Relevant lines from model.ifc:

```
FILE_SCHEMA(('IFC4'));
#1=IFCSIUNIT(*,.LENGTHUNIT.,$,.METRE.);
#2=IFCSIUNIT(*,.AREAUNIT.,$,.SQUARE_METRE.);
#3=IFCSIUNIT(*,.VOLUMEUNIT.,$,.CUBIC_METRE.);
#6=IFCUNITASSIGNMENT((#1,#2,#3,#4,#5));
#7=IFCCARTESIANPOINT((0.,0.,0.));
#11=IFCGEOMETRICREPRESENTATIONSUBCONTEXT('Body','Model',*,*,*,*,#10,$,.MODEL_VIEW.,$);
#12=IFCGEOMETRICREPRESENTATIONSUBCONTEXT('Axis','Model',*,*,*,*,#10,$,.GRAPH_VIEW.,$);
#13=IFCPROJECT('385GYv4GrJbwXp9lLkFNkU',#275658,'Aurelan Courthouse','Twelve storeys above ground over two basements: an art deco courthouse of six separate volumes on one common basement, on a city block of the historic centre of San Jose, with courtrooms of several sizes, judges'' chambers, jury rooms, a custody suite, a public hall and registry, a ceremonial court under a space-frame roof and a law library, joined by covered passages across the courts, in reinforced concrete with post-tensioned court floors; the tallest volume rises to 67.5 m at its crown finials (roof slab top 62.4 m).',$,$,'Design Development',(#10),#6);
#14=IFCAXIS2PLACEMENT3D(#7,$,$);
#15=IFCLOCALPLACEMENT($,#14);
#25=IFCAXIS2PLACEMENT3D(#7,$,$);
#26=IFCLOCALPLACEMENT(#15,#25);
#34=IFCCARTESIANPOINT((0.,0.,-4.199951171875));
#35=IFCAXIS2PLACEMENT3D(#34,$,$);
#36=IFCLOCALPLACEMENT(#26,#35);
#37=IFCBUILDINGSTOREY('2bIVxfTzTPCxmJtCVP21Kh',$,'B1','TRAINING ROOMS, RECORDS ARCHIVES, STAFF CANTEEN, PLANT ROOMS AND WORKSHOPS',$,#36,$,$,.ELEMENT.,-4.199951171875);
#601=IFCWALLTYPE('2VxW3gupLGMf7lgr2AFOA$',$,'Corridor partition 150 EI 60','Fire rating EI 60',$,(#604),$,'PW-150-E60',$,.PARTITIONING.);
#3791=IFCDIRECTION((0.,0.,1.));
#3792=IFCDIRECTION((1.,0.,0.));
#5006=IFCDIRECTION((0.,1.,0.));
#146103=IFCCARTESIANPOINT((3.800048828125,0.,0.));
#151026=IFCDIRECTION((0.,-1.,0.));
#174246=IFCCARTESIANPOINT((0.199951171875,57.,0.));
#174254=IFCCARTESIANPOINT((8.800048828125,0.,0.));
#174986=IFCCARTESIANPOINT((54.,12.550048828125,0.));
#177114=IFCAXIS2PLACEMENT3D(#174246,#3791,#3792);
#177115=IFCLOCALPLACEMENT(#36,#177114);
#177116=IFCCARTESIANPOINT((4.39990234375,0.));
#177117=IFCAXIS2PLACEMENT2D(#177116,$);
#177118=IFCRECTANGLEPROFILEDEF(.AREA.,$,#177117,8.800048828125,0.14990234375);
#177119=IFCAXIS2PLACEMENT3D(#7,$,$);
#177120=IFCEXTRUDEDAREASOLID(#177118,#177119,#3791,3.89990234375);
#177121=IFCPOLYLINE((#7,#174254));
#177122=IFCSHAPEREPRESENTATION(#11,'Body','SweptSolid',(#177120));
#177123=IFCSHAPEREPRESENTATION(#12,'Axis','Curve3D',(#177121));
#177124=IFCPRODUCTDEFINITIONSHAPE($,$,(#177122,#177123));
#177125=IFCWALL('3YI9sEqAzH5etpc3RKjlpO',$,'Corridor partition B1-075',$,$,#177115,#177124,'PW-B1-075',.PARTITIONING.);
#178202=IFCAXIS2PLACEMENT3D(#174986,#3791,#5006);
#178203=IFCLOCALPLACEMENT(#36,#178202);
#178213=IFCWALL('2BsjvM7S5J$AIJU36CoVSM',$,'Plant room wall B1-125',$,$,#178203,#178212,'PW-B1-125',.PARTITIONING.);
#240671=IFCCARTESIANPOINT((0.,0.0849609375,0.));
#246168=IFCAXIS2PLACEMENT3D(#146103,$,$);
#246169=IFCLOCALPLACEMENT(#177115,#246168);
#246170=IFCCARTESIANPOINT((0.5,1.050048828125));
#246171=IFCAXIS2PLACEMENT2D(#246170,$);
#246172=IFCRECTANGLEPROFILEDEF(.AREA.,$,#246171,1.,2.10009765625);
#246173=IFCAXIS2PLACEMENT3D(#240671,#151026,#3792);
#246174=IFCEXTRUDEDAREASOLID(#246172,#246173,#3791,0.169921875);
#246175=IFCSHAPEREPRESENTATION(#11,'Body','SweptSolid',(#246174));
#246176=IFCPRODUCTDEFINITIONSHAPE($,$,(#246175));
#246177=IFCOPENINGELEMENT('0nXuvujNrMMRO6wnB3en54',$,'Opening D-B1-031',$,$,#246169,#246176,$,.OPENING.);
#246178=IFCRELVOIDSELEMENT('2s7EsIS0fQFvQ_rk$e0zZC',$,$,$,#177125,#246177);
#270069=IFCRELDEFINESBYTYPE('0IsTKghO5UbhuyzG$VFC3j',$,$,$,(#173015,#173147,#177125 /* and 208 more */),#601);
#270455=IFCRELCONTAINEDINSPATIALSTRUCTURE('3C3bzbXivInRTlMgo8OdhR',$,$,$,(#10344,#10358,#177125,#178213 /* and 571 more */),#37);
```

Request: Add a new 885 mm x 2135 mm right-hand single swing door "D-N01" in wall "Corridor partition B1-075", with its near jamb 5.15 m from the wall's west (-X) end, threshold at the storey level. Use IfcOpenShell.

```python
import numpy as np
import ifcopenshell
import ifcopenshell.api.feature
import ifcopenshell.api.geometry
import ifcopenshell.api.root
import ifcopenshell.api.spatial
import ifcopenshell.geom
import ifcopenshell.util.element
import ifcopenshell.util.placement
import ifcopenshell.util.representation
import ifcopenshell.util.shape
import ifcopenshell.util.unit

model = ifcopenshell.open("model.ifc")
unit_scale = ifcopenshell.util.unit.calculate_unit_scale(model)
settings = ifcopenshell.geom.settings()


def volume(element):
    """Net volume in cubic metres, openings subtracted."""
    shape = ifcopenshell.geom.create_shape(settings, element)
    return ifcopenshell.util.shape.get_volume(shape.geometry)


wall = model.by_guid("3YI9sEqAzH5etpc3RKjlpO")
storey = ifcopenshell.util.element.get_container(wall, ifc_class="IfcBuildingStorey")
context = ifcopenshell.util.representation.get_context(model, "Model", "Body", "MODEL_VIEW")
before = volume(wall)

width, height, from_end, sill = 0.885, 2.135, 5.15, 0.0  # metres

# The wall runs along its own X axis, and the end named is its -X end.
wall_shape = ifcopenshell.geom.create_shape(settings, wall)
x, y, z = ifcopenshell.util.shape.get_vertices(wall_shape.geometry).T
start = x.min() + from_end
face, thickness = float(y.min()), float(y.max() - y.min())
wall_matrix = ifcopenshell.util.placement.get_local_placement(wall.ObjectPlacement)
level = ifcopenshell.util.placement.get_local_placement(storey.ObjectPlacement)[2, 3]


def in_wall(x, y):
    """Placement at x, y metres in the wall's axes, at sill height."""
    matrix = wall_matrix.copy()
    matrix[:, 3] = wall_matrix @ np.array([x / unit_scale, y / unit_scale, 0.0, 1.0])
    matrix[2, 3] = level + sill / unit_scale
    return matrix


# Opening: a box that overshoots both wall faces by 50 mm.
opening = ifcopenshell.api.root.create_entity(model, ifc_class="IfcOpeningElement", predefined_type="OPENING")
box = ifcopenshell.api.geometry.add_wall_representation(
    model, context=context, length=width, height=height, thickness=thickness + 0.1
)
ifcopenshell.api.geometry.assign_representation(model, product=opening, representation=box)
ifcopenshell.api.geometry.edit_object_placement(model, product=opening, matrix=in_wall(start, face - 0.05), is_si=False)
ifcopenshell.api.feature.add_feature(model, feature=opening, element=wall)

door = ifcopenshell.api.root.create_entity(model, ifc_class="IfcDoor", name="D-N01", predefined_type="DOOR")
door.OverallWidth, door.OverallHeight = width / unit_scale, height / unit_scale
door.OperationType = "SINGLE_SWING_RIGHT"
body = ifcopenshell.api.geometry.add_door_representation(
    model,
    context=context,
    overall_width=door.OverallWidth,
    overall_height=door.OverallHeight,
    operation_type="SINGLE_SWING_RIGHT",
    lining_properties={"LiningDepth": thickness / unit_scale, "ThresholdDepth": thickness / unit_scale},
)
ifcopenshell.api.geometry.assign_representation(model, product=door, representation=body)
ifcopenshell.api.spatial.assign_container(model, products=[door], relating_structure=storey)
ifcopenshell.api.feature.add_filling(model, opening=opening, element=door)

# The lining spans the wall, so the door starts at the wall face.
ifcopenshell.api.geometry.edit_object_placement(model, product=door, matrix=in_wall(start, face), is_si=False)

after = volume(wall)

print(f"wall volume {before:.3f} -> {after:.3f} m3")

model.write("model_rev.ifc")
```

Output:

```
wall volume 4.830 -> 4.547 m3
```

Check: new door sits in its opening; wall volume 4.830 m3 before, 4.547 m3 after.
